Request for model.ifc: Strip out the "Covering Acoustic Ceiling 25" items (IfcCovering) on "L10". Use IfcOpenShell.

First a look at what the model holds.

```python
import ifcopenshell
import ifcopenshell.util.element

model = ifcopenshell.open("model.ifc")
print(model.schema)
storey = next(s for s in model.by_type("IfcBuildingStorey") if s.Name == "L10")
coverings = [e for e in ifcopenshell.util.element.get_decomposition(storey) if e.is_a("IfcCovering")]
seen = {}
for e in coverings:
    element_type = ifcopenshell.util.element.get_type(e)
    name = element_type.Name if element_type not in (None, e) else None
    seen[name] = seen.get(name, 0) + 1
for name, count in sorted(seen.items(), key=str):
    print(count, "x", name)
```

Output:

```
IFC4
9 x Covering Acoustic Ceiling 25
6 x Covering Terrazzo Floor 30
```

```python
import ifcopenshell
import ifcopenshell.api.root
import ifcopenshell.util.element

model = ifcopenshell.open("model.ifc")

storey = next(s for s in model.by_type("IfcBuildingStorey") if s.Name == "L10")
coverings = [e for e in ifcopenshell.util.element.get_decomposition(storey) if e.is_a("IfcCovering")]
targets = [e for e in coverings if (t := ifcopenshell.util.element.get_type(e)) not in (None, e) and t.Name == "Covering Acoustic Ceiling 25"]

for e in targets:
    ifcopenshell.api.root.remove_product(model, product=e)
print(len(targets), "removed")

model.write("model_v2.ifc")
```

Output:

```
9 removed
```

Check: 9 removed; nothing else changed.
